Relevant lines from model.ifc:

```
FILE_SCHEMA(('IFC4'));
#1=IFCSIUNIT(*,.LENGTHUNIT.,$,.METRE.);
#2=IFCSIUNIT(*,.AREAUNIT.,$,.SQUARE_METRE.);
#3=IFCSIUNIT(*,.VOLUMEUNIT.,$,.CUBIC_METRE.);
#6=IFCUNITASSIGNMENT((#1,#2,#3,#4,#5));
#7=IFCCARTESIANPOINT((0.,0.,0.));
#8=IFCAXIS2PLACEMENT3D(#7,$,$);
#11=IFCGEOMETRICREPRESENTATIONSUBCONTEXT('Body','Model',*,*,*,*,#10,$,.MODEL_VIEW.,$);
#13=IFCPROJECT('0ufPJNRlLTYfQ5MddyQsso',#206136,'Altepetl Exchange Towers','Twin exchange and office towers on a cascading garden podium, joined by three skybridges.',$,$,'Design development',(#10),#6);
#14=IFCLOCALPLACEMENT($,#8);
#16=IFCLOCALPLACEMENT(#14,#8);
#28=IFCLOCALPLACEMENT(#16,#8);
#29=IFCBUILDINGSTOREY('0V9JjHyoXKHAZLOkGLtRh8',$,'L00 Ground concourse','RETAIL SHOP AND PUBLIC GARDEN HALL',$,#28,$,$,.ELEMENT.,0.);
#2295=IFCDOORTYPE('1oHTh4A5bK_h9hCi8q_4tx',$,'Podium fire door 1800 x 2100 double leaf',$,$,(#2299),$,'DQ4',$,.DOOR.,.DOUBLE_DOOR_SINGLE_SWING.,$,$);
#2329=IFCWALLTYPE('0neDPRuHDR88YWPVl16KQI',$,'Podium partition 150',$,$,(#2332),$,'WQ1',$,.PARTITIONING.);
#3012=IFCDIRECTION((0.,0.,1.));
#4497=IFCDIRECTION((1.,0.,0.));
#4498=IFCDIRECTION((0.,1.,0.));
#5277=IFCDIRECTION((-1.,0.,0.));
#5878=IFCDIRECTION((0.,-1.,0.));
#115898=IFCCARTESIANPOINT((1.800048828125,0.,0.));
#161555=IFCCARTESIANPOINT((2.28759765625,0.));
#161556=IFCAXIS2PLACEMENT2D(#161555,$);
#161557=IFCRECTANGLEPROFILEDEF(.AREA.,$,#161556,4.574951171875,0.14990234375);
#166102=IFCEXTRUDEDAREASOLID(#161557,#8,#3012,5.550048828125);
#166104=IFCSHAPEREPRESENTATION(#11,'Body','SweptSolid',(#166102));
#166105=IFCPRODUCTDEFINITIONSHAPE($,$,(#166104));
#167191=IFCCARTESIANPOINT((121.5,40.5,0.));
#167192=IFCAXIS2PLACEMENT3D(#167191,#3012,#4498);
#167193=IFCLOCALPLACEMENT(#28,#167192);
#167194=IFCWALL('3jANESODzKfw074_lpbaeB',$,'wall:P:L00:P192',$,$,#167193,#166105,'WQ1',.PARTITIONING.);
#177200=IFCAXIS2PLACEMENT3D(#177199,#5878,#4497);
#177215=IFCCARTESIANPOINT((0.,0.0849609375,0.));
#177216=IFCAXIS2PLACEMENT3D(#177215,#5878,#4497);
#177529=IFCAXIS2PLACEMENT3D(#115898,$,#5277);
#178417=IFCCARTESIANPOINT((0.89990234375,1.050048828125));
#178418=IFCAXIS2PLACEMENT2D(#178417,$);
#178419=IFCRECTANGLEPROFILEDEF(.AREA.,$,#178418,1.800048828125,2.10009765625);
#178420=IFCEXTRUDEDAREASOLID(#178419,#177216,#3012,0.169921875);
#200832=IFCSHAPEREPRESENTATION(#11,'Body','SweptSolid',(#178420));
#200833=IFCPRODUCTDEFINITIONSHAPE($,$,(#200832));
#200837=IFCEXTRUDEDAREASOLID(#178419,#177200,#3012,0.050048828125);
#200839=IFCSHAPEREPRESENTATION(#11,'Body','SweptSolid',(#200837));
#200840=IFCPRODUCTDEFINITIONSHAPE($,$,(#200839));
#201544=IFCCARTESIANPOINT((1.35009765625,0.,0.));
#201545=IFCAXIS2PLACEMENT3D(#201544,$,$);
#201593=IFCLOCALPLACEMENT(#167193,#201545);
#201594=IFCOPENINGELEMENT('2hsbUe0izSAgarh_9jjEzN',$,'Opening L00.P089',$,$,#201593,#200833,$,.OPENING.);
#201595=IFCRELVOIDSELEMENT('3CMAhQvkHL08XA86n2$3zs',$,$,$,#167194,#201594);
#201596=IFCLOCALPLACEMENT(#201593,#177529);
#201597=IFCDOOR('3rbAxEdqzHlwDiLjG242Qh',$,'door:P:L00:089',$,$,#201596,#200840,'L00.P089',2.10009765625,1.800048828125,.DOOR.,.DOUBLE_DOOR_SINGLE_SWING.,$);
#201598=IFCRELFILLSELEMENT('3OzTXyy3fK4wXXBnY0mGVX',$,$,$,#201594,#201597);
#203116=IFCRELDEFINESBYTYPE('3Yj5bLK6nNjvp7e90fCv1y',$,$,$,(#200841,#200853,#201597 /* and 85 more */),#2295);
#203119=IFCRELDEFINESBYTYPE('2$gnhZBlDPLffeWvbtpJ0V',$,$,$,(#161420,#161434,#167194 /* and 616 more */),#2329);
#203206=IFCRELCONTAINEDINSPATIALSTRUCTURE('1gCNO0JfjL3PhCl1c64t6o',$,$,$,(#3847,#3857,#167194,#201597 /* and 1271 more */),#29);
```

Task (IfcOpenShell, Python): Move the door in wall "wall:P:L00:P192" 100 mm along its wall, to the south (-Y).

```python
import ifcopenshell
import ifcopenshell.api.geometry
import ifcopenshell.util.placement

model = ifcopenshell.open("model.ifc")

door = model.by_guid("3rbAxEdqzHlwDiLjG242Qh")
opening = door.FillsVoids[0].RelatingOpeningElement
wall = opening.VoidsElements[0].RelatingBuildingElement

wall_matrix = ifcopenshell.util.placement.get_local_placement(wall.ObjectPlacement)
shift = wall_matrix[:3, 0] * -0.1
before = ifcopenshell.util.placement.get_local_placement(door.ObjectPlacement)[:3, 3].copy()

# The door is placed relative to its opening, so it follows when the opening moves.
matrix = ifcopenshell.util.placement.get_local_placement(opening.ObjectPlacement)
matrix[:3, 3] += shift
ifcopenshell.api.geometry.edit_object_placement(
    model, product=opening, matrix=matrix, is_si=False, should_transform_children=True
)

after = ifcopenshell.util.placement.get_local_placement(door.ObjectPlacement)[:3, 3]
print("door moved by", (after - before).round(3) + 0.0)

model.write("model_edited.ifc")
```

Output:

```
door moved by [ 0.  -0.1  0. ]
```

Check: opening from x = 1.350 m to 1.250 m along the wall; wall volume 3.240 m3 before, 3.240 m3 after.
